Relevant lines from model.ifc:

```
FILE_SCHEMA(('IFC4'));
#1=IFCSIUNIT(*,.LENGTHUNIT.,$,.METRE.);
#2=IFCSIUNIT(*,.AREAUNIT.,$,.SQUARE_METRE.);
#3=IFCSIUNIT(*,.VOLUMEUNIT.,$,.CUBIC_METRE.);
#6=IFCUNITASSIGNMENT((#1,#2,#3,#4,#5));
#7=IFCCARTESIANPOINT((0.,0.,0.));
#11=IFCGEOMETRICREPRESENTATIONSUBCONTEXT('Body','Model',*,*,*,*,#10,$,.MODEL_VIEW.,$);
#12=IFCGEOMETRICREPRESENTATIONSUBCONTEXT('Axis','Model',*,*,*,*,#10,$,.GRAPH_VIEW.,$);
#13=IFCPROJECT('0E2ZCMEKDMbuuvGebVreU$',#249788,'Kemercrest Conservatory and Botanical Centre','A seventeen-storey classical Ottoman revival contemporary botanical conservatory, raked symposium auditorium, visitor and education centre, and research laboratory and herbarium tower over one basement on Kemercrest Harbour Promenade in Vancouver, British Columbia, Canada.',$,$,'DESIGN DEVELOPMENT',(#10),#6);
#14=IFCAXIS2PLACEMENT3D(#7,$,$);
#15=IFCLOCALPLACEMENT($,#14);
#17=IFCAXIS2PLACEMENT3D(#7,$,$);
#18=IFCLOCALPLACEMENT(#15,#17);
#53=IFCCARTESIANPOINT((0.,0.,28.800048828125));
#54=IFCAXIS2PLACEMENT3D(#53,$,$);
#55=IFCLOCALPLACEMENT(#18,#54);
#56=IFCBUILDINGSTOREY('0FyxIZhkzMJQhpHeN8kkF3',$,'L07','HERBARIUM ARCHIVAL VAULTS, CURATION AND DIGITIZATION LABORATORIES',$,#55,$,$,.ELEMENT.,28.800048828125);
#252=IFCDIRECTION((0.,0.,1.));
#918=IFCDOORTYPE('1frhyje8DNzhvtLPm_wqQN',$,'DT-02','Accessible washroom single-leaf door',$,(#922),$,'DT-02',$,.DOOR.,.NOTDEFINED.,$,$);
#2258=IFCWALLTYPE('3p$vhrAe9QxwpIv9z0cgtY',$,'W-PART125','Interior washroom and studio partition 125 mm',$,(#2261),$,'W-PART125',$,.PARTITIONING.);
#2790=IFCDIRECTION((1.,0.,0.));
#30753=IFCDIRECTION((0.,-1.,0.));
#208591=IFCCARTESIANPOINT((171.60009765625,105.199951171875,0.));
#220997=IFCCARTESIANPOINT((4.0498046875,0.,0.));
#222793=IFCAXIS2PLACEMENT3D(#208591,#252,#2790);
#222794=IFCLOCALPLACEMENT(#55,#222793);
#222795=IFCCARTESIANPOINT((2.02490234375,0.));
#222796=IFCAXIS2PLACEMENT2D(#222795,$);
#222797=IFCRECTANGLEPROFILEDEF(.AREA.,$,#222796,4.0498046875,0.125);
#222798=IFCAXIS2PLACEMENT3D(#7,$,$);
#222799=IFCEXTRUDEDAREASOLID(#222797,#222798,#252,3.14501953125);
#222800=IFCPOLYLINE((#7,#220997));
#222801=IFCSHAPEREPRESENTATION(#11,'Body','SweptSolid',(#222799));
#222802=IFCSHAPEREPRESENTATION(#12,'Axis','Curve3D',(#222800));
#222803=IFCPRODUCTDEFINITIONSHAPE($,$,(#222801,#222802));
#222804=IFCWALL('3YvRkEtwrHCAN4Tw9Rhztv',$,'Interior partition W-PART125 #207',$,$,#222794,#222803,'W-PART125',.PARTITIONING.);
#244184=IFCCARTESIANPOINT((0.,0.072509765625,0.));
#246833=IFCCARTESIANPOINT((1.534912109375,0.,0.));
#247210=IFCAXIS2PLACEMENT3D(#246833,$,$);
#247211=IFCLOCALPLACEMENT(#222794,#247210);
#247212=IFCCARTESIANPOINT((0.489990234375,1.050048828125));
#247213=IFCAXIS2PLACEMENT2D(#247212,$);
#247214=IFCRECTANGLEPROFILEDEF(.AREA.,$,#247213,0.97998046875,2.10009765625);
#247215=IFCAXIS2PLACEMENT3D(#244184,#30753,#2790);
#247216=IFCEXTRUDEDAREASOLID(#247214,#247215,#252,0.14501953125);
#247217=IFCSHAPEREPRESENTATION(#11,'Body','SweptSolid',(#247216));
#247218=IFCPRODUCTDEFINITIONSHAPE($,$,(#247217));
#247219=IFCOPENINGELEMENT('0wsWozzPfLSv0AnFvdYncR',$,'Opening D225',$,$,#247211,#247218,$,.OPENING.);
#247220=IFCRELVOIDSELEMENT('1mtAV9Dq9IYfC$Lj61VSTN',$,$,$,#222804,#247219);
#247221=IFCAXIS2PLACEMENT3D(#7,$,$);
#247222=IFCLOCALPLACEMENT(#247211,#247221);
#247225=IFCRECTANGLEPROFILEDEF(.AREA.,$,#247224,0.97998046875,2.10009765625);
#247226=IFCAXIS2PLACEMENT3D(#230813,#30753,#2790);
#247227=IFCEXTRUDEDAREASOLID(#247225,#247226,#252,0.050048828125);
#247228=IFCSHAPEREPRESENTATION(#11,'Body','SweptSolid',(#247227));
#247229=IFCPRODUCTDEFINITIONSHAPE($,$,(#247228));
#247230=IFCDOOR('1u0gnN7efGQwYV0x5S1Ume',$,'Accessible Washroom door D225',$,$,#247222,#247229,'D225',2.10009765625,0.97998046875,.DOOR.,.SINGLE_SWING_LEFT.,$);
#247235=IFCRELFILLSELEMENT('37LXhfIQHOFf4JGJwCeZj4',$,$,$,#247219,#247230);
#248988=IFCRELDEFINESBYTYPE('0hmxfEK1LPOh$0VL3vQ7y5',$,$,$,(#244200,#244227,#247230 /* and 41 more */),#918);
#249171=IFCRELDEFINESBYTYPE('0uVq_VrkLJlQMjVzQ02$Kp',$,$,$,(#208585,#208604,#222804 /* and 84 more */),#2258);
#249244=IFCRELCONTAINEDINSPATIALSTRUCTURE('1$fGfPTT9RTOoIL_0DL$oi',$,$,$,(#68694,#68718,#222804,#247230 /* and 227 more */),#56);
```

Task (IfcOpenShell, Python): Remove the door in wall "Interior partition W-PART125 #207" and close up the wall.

```python
import ifcopenshell
import ifcopenshell.api.feature
import ifcopenshell.api.root
import ifcopenshell.geom
import ifcopenshell.util.shape

model = ifcopenshell.open("model.ifc")
settings = ifcopenshell.geom.settings()


def volume(element):
    """Net volume in cubic metres, openings subtracted."""
    shape = ifcopenshell.geom.create_shape(settings, element)
    return ifcopenshell.util.shape.get_volume(shape.geometry)


door = model.by_guid("1u0gnN7efGQwYV0x5S1Ume")
opening = door.FillsVoids[0].RelatingOpeningElement
wall = opening.VoidsElements[0].RelatingBuildingElement
before = volume(wall)

ifcopenshell.api.root.remove_product(model, product=door)
ifcopenshell.api.feature.remove_feature(model, feature=opening)

after = volume(wall)

print(f"wall volume {before:.3f} -> {after:.3f} m3")

model.write("model_edited.ifc")
```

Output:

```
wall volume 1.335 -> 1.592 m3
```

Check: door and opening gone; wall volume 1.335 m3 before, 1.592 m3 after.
